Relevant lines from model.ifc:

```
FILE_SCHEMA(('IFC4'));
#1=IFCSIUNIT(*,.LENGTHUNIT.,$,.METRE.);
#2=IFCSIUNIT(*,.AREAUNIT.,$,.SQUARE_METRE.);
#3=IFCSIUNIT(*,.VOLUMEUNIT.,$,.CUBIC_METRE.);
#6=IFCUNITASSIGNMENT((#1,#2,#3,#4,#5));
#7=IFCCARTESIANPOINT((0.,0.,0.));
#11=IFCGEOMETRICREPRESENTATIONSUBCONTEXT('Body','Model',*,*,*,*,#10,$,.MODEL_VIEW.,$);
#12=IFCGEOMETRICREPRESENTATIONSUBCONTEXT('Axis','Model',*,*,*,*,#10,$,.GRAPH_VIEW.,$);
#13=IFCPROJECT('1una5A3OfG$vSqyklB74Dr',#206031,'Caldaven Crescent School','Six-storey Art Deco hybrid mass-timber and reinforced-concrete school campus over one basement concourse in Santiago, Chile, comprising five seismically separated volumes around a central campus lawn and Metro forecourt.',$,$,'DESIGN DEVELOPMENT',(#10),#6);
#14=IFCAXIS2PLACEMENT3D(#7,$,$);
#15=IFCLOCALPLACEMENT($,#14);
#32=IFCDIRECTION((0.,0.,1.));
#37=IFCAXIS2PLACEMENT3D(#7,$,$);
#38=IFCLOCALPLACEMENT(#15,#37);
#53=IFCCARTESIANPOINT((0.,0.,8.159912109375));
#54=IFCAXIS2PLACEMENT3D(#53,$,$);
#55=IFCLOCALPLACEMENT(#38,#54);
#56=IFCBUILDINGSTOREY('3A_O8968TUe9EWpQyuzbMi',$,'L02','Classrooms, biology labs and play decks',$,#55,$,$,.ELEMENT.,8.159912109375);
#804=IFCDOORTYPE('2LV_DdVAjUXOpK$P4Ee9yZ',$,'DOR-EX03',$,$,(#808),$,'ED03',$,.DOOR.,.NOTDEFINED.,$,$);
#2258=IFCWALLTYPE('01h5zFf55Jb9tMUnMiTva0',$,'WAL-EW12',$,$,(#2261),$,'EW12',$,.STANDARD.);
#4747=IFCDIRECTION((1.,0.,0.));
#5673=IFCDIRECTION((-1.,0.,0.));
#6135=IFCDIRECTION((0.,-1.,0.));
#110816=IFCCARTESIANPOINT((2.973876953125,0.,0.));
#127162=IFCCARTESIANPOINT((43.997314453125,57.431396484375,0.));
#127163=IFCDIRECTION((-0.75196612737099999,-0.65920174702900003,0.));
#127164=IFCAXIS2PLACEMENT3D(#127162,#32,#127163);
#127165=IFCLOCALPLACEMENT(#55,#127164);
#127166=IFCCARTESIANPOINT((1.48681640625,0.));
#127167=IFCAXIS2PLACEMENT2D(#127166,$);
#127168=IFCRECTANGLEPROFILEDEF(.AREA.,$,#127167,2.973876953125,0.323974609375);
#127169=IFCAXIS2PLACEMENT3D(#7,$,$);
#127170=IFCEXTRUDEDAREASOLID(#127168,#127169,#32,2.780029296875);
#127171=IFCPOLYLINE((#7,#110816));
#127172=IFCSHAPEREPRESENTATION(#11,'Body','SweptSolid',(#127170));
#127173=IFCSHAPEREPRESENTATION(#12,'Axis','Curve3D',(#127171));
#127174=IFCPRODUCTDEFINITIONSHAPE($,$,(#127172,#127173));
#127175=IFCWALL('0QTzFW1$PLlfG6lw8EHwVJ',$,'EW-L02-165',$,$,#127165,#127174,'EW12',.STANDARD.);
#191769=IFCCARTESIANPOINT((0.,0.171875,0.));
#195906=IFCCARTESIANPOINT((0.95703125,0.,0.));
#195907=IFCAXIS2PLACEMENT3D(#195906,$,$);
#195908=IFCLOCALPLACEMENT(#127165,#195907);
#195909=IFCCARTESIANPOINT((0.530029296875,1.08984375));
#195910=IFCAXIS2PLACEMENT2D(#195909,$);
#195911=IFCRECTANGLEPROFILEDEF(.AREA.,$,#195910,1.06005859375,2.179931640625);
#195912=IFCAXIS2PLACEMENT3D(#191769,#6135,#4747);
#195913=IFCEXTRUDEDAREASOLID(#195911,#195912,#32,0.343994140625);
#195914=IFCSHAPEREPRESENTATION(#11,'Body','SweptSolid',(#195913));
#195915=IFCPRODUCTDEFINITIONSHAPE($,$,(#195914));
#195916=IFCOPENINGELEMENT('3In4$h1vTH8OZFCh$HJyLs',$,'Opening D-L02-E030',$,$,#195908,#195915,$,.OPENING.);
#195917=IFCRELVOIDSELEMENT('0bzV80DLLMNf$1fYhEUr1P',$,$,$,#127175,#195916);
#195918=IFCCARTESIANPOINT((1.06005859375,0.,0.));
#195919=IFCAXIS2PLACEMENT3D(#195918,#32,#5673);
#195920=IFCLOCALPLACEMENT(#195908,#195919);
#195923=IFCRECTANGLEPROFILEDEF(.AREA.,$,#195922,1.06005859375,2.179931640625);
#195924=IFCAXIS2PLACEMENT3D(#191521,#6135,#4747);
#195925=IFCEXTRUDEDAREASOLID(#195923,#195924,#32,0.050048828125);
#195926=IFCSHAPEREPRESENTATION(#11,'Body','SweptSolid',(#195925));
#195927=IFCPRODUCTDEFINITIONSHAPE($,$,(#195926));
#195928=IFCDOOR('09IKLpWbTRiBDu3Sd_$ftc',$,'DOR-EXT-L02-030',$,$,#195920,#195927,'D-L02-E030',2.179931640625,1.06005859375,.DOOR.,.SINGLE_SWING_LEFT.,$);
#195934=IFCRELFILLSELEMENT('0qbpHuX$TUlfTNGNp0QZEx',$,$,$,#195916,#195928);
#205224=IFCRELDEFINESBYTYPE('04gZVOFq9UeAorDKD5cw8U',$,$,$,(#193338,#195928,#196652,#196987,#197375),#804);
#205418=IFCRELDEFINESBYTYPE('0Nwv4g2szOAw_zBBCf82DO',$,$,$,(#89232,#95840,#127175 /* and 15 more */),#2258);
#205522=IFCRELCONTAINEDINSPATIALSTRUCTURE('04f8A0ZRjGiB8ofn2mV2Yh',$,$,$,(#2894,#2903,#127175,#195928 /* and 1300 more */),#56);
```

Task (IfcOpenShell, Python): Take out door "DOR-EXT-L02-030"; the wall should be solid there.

```python
import ifcopenshell
import ifcopenshell.api.feature
import ifcopenshell.api.root
import ifcopenshell.geom
import ifcopenshell.util.shape

model = ifcopenshell.open("model.ifc")
settings = ifcopenshell.geom.settings()


def volume(element):
    """Net volume in cubic metres, openings subtracted."""
    shape = ifcopenshell.geom.create_shape(settings, element)
    return ifcopenshell.util.shape.get_volume(shape.geometry)


door = model.by_guid("09IKLpWbTRiBDu3Sd_$ftc")
opening = door.FillsVoids[0].RelatingOpeningElement
wall = opening.VoidsElements[0].RelatingBuildingElement
before = volume(wall)

ifcopenshell.api.root.remove_product(model, product=door)
ifcopenshell.api.feature.remove_feature(model, feature=opening)

after = volume(wall)

print(f"wall volume {before:.3f} -> {after:.3f} m3")

model.write("model_edited.ifc")
```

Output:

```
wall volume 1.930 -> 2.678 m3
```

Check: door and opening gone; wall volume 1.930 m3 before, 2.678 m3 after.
